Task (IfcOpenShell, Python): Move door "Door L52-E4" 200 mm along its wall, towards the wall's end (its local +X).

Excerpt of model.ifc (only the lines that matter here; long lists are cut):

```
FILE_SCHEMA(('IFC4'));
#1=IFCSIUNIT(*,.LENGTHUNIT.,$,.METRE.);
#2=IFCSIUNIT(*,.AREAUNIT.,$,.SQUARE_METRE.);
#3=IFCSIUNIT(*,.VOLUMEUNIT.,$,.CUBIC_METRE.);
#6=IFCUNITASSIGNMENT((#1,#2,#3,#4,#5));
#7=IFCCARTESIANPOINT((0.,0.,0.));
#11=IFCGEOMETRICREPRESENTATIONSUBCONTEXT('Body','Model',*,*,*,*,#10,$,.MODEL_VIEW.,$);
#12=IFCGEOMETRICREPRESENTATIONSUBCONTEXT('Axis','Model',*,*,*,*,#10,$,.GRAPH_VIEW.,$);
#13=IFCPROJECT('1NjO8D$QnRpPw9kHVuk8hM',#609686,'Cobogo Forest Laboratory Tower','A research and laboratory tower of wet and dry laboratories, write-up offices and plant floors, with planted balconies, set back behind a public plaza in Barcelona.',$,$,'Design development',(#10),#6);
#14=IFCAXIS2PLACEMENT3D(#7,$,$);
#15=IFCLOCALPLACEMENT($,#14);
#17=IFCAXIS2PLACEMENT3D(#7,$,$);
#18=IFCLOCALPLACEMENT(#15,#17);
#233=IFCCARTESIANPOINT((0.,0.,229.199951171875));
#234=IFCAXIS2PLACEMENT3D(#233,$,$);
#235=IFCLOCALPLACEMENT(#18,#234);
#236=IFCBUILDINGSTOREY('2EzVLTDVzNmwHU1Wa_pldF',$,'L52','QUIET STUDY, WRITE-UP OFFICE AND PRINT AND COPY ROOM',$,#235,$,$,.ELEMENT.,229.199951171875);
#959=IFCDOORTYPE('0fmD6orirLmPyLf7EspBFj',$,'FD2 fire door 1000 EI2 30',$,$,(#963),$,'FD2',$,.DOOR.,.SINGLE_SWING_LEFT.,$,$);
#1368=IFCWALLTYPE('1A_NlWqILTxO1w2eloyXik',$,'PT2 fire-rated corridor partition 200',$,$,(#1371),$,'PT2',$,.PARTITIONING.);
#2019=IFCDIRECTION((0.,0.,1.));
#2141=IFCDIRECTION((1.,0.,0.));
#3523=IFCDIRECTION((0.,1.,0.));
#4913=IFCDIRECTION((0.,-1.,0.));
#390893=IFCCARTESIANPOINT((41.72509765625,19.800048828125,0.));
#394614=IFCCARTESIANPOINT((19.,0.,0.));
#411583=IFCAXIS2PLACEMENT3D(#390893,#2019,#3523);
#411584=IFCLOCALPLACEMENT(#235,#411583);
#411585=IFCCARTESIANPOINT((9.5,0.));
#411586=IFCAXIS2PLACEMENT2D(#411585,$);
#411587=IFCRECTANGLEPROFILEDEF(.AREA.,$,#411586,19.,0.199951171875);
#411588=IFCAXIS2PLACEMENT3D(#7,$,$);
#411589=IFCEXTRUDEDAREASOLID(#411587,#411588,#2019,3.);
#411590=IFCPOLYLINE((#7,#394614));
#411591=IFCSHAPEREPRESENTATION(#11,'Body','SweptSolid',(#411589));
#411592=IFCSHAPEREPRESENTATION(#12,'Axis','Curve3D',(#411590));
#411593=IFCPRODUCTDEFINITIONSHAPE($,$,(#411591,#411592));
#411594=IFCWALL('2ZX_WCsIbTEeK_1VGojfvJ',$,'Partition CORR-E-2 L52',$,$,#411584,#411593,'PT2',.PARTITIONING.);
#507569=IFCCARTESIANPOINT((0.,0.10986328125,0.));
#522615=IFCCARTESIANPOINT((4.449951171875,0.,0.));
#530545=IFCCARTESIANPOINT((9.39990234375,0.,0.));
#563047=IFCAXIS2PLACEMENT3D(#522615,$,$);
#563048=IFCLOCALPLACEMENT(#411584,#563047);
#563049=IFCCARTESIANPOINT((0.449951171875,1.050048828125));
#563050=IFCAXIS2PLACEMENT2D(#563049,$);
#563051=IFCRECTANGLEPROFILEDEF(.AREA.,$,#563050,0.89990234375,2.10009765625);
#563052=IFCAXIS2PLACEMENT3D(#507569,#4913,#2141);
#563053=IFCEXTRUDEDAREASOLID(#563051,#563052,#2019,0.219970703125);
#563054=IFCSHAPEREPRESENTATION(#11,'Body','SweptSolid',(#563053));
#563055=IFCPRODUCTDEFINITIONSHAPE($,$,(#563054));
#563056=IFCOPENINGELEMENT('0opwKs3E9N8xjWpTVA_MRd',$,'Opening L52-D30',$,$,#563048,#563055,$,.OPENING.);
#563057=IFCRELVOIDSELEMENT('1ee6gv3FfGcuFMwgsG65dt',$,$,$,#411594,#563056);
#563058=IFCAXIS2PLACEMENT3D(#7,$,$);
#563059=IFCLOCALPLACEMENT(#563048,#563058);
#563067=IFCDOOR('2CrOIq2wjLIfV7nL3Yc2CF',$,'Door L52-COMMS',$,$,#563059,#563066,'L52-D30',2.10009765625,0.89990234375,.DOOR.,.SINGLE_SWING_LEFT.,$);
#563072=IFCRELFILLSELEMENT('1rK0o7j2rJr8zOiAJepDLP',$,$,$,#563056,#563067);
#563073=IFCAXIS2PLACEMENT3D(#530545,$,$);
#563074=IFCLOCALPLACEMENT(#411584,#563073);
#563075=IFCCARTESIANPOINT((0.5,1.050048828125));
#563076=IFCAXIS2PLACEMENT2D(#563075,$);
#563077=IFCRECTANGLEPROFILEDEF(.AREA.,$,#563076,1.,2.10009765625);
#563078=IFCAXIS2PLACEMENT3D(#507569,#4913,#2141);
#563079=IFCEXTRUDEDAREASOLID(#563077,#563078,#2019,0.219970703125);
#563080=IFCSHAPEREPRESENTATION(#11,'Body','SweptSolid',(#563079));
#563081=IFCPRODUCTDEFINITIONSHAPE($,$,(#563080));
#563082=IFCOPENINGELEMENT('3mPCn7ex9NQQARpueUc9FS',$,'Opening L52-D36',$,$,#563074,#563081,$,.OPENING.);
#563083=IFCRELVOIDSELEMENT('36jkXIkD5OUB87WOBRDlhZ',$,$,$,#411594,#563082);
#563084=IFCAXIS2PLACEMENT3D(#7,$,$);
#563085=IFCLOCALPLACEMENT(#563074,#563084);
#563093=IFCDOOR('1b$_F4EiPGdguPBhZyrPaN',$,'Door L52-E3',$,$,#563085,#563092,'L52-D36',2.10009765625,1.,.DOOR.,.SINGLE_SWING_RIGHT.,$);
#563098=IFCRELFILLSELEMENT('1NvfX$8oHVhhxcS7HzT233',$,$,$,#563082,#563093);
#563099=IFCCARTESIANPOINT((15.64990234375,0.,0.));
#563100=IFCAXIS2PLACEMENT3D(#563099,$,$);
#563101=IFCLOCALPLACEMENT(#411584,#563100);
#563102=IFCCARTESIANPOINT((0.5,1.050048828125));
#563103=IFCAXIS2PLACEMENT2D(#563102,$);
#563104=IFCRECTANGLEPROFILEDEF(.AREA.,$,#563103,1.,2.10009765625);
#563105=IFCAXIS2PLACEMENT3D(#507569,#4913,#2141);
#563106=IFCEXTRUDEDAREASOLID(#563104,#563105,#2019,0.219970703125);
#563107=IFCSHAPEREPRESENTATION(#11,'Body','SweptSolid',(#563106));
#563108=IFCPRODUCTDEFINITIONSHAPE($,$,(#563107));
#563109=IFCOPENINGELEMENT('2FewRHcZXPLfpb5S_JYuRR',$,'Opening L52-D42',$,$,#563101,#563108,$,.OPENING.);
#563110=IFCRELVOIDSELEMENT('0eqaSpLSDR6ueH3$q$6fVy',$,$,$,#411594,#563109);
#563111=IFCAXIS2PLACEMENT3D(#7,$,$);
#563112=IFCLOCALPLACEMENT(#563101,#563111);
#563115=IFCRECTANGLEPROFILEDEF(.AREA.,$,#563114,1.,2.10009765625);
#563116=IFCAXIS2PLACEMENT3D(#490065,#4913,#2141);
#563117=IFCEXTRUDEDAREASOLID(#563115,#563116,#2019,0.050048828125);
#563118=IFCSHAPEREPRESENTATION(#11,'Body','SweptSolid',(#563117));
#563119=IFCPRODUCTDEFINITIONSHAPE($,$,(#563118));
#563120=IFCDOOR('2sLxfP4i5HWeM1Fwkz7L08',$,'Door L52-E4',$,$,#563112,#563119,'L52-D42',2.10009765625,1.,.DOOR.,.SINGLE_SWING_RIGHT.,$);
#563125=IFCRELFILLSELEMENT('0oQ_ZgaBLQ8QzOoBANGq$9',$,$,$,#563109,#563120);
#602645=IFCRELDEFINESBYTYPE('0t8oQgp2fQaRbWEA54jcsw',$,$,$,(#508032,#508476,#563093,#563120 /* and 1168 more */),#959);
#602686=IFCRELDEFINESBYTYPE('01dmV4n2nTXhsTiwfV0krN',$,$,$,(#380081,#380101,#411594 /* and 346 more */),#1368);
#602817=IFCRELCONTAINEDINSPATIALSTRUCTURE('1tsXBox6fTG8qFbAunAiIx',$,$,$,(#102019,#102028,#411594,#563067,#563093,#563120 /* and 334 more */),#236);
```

```python
import ifcopenshell
import ifcopenshell.api.geometry
import ifcopenshell.util.placement

model = ifcopenshell.open("model.ifc")

door = model.by_guid("2sLxfP4i5HWeM1Fwkz7L08")
opening = door.FillsVoids[0].RelatingOpeningElement
wall = opening.VoidsElements[0].RelatingBuildingElement

wall_matrix = ifcopenshell.util.placement.get_local_placement(wall.ObjectPlacement)
shift = wall_matrix[:3, 0] * 0.2
before = ifcopenshell.util.placement.get_local_placement(door.ObjectPlacement)[:3, 3].copy()

# The door is placed relative to its opening, so it follows when the opening moves.
matrix = ifcopenshell.util.placement.get_local_placement(opening.ObjectPlacement)
matrix[:3, 3] += shift
ifcopenshell.api.geometry.edit_object_placement(
    model, product=opening, matrix=matrix, is_si=False, should_transform_children=True
)

after = ifcopenshell.util.placement.get_local_placement(door.ObjectPlacement)[:3, 3]
print("door moved by", (after - before).round(3) + 0.0)

model.write("model_rev.ifc")
```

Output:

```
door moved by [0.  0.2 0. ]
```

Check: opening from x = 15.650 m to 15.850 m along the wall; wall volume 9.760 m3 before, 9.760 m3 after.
